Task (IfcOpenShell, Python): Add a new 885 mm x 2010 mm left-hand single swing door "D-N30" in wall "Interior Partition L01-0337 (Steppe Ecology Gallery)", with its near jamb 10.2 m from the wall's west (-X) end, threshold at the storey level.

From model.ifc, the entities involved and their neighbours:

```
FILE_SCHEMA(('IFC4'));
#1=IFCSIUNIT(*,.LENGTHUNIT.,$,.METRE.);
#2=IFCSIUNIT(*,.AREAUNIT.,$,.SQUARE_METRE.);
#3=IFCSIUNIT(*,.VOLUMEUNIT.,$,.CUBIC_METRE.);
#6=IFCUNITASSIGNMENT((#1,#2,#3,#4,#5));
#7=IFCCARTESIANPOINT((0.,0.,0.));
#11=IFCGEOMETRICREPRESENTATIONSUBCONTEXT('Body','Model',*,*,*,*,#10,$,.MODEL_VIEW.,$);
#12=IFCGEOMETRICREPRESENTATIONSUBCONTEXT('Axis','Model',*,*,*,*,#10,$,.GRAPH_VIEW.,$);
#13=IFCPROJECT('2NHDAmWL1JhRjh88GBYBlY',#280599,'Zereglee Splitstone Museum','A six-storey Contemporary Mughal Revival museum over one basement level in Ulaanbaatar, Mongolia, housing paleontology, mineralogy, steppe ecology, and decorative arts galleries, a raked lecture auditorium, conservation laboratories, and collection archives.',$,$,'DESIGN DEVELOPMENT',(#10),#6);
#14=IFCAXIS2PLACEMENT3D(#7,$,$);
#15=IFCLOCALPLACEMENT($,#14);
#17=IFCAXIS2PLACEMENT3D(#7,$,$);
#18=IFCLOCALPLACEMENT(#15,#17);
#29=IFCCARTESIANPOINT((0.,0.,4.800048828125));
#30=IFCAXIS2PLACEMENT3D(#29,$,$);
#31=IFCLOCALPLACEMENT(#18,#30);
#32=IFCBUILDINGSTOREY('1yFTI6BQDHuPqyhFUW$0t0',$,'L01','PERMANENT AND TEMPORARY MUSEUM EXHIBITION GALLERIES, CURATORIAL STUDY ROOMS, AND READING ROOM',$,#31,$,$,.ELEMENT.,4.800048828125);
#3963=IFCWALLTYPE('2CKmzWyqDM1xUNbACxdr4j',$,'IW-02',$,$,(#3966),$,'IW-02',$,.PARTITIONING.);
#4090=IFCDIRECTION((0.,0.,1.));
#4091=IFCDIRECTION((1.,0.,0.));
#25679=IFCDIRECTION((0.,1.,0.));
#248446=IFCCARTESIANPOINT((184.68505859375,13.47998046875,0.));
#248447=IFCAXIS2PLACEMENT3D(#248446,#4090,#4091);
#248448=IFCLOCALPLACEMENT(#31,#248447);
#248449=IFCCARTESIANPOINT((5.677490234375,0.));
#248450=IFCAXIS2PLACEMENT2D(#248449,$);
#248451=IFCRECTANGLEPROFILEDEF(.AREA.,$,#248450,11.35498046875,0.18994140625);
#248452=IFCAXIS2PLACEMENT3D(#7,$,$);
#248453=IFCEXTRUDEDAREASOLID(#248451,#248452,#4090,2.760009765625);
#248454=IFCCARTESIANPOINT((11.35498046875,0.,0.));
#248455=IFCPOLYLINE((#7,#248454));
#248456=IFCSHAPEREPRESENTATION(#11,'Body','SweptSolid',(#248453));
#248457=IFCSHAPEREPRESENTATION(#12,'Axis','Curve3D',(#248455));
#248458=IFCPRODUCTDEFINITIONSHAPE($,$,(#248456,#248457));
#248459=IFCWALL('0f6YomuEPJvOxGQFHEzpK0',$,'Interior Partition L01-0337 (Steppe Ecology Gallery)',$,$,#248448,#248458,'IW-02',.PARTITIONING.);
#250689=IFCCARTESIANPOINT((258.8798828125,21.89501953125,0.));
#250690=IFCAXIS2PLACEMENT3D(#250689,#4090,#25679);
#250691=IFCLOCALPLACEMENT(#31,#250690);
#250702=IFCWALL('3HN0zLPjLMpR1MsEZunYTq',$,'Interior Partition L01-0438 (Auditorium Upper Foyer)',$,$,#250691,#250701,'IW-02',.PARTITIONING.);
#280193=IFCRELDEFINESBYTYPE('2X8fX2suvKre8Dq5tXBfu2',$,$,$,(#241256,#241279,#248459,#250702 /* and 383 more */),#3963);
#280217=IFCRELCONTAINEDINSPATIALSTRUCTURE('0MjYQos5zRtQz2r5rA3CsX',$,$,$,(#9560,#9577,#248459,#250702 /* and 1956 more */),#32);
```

```python
import numpy as np
import ifcopenshell
import ifcopenshell.api.feature
import ifcopenshell.api.geometry
import ifcopenshell.api.root
import ifcopenshell.api.spatial
import ifcopenshell.geom
import ifcopenshell.util.element
import ifcopenshell.util.placement
import ifcopenshell.util.representation
import ifcopenshell.util.shape
import ifcopenshell.util.unit

model = ifcopenshell.open("model.ifc")
unit_scale = ifcopenshell.util.unit.calculate_unit_scale(model)
settings = ifcopenshell.geom.settings()


def volume(element):
    """Net volume in cubic metres, openings subtracted."""
    shape = ifcopenshell.geom.create_shape(settings, element)
    return ifcopenshell.util.shape.get_volume(shape.geometry)


wall = model.by_guid("0f6YomuEPJvOxGQFHEzpK0")
storey = ifcopenshell.util.element.get_container(wall, ifc_class="IfcBuildingStorey")
context = ifcopenshell.util.representation.get_context(model, "Model", "Body", "MODEL_VIEW")
before = volume(wall)

width, height, from_end, sill = 0.885, 2.01, 10.2, 0.0  # metres

# The wall runs along its own X axis, and the end named is its -X end.
wall_shape = ifcopenshell.geom.create_shape(settings, wall)
x, y, z = ifcopenshell.util.shape.get_vertices(wall_shape.geometry).T
start = x.min() + from_end
face, thickness = float(y.min()), float(y.max() - y.min())
wall_matrix = ifcopenshell.util.placement.get_local_placement(wall.ObjectPlacement)
level = ifcopenshell.util.placement.get_local_placement(storey.ObjectPlacement)[2, 3]


def in_wall(x, y):
    """Placement at x, y metres in the wall's axes, at sill height."""
    matrix = wall_matrix.copy()
    matrix[:, 3] = wall_matrix @ np.array([x / unit_scale, y / unit_scale, 0.0, 1.0])
    matrix[2, 3] = level + sill / unit_scale
    return matrix


# Opening: a box that overshoots both wall faces by 50 mm.
opening = ifcopenshell.api.root.create_entity(model, ifc_class="IfcOpeningElement", predefined_type="OPENING")
box = ifcopenshell.api.geometry.add_wall_representation(
    model, context=context, length=width, height=height, thickness=thickness + 0.1
)
ifcopenshell.api.geometry.assign_representation(model, product=opening, representation=box)
ifcopenshell.api.geometry.edit_object_placement(model, product=opening, matrix=in_wall(start, face - 0.05), is_si=False)
ifcopenshell.api.feature.add_feature(model, feature=opening, element=wall)

door = ifcopenshell.api.root.create_entity(model, ifc_class="IfcDoor", name="D-N30", predefined_type="DOOR")
door.OverallWidth, door.OverallHeight = width / unit_scale, height / unit_scale
door.OperationType = "SINGLE_SWING_LEFT"
body = ifcopenshell.api.geometry.add_door_representation(
    model,
    context=context,
    overall_width=door.OverallWidth,
    overall_height=door.OverallHeight,
    operation_type="SINGLE_SWING_LEFT",
    lining_properties={"LiningDepth": thickness / unit_scale, "ThresholdDepth": thickness / unit_scale},
)
ifcopenshell.api.geometry.assign_representation(model, product=door, representation=body)
ifcopenshell.api.spatial.assign_container(model, products=[door], relating_structure=storey)
ifcopenshell.api.feature.add_filling(model, opening=opening, element=door)

# The lining spans the wall, so the door starts at the wall face.
ifcopenshell.api.geometry.edit_object_placement(model, product=door, matrix=in_wall(start, face), is_si=False)

after = volume(wall)

print(f"wall volume {before:.3f} -> {after:.3f} m3")

model.write("model-out.ifc")
```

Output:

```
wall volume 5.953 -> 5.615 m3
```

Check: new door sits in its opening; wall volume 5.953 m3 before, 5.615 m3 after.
